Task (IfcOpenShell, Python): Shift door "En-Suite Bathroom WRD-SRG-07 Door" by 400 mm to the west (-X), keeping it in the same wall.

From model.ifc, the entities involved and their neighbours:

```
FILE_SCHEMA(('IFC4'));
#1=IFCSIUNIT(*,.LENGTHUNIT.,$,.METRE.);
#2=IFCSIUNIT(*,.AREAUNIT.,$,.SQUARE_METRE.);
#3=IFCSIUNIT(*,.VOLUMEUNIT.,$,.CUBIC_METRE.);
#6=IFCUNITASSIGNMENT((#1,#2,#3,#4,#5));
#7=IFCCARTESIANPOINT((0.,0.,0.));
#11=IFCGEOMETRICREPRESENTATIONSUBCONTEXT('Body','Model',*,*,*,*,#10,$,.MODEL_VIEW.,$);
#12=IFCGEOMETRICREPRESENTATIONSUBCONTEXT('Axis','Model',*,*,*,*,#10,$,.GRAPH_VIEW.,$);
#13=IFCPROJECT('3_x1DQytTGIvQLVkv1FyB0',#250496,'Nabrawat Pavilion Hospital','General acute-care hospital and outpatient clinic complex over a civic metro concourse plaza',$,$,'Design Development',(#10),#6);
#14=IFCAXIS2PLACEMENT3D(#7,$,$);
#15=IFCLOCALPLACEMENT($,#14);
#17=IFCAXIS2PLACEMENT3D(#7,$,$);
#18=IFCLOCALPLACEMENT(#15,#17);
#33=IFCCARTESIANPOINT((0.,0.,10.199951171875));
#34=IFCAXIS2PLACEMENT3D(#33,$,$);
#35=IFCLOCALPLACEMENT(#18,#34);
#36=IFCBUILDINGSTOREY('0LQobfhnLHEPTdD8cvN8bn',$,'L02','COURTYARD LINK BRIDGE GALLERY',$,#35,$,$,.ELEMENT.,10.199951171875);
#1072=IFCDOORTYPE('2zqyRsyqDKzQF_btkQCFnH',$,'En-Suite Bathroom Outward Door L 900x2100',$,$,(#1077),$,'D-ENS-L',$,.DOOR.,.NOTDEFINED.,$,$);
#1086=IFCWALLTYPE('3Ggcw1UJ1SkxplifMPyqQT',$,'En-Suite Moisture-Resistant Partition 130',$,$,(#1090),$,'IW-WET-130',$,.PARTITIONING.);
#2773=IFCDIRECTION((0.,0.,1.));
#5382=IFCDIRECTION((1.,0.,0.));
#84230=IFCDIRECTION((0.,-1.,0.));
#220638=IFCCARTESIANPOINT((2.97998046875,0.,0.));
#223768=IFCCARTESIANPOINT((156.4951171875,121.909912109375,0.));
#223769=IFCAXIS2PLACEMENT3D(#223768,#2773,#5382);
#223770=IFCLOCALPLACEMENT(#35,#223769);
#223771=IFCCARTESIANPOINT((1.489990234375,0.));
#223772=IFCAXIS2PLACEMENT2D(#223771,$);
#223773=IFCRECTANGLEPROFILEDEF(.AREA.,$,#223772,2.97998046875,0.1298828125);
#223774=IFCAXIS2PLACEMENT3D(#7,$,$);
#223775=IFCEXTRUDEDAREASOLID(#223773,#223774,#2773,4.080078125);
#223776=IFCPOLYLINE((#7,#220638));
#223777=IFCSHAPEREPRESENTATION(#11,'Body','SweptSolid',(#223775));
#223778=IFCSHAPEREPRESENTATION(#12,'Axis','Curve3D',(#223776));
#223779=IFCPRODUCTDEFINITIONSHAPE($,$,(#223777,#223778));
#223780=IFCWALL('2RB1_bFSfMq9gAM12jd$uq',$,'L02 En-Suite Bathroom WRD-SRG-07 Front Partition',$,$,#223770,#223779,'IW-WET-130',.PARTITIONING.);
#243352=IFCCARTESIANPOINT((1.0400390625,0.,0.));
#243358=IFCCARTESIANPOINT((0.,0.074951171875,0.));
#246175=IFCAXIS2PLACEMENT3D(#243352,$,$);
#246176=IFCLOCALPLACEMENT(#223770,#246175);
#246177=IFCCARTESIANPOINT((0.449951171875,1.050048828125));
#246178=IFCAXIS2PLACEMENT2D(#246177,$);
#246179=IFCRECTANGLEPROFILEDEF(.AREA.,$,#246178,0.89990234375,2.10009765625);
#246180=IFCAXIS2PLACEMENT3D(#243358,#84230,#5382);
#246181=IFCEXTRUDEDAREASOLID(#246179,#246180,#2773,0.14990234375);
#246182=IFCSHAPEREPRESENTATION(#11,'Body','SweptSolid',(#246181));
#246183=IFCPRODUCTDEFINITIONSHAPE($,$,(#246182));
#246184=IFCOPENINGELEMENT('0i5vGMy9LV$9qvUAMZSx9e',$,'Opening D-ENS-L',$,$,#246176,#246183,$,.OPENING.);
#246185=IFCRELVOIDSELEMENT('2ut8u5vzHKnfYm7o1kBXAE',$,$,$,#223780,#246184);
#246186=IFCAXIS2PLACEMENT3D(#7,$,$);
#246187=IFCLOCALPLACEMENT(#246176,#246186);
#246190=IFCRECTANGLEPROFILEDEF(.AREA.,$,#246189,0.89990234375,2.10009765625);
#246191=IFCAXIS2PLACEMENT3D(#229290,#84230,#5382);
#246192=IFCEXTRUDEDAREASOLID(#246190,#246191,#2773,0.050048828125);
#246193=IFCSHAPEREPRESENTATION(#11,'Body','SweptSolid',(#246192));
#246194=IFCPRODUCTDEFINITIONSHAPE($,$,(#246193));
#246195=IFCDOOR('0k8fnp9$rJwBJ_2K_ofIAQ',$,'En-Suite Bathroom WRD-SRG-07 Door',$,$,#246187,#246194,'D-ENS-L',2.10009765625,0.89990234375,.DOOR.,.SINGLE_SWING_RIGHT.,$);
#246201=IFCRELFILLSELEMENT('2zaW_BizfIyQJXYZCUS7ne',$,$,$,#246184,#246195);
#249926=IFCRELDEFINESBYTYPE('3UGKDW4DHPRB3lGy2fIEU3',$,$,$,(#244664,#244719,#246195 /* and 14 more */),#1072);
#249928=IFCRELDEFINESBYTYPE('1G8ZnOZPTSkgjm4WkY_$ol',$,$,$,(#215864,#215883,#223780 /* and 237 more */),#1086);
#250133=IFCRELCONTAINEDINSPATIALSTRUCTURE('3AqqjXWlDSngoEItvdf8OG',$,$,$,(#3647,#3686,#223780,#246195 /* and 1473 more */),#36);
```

```python
import ifcopenshell
import ifcopenshell.api.geometry
import ifcopenshell.util.placement

model = ifcopenshell.open("model.ifc")

door = model.by_id(246195)
opening = door.FillsVoids[0].RelatingOpeningElement
wall = opening.VoidsElements[0].RelatingBuildingElement

wall_matrix = ifcopenshell.util.placement.get_local_placement(wall.ObjectPlacement)
shift = wall_matrix[:3, 0] * -0.4
before = ifcopenshell.util.placement.get_local_placement(door.ObjectPlacement)[:3, 3].copy()

# The door is placed relative to its opening, so it follows when the opening moves.
matrix = ifcopenshell.util.placement.get_local_placement(opening.ObjectPlacement)
matrix[:3, 3] += shift
ifcopenshell.api.geometry.edit_object_placement(
    model, product=opening, matrix=matrix, is_si=False, should_transform_children=True
)

after = ifcopenshell.util.placement.get_local_placement(door.ObjectPlacement)[:3, 3]
print("door moved by", (after - before).round(3) + 0.0)

model.write("model_v2.ifc")
```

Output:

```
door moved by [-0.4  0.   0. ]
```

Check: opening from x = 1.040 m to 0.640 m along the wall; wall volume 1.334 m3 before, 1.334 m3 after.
